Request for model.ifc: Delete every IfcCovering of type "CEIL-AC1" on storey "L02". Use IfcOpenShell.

First a look at what the model holds.

```python
import ifcopenshell
import ifcopenshell.util.element

model = ifcopenshell.open("model.ifc")
print(model.schema)
storey = next(s for s in model.by_type("IfcBuildingStorey") if s.Name == "L02")
coverings = [e for e in ifcopenshell.util.element.get_decomposition(storey) if e.is_a("IfcCovering")]
seen = {}
for e in coverings:
    element_type = ifcopenshell.util.element.get_type(e)
    name = element_type.Name if element_type not in (None, e) else None
    seen[name] = seen.get(name, 0) + 1
for name, count in sorted(seen.items(), key=str):
    print(count, "x", name)
```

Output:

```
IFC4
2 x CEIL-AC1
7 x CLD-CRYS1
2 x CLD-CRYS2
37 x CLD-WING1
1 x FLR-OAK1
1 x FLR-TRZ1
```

```python
import ifcopenshell
import ifcopenshell.api.root
import ifcopenshell.util.element

model = ifcopenshell.open("model.ifc")

storey = next(s for s in model.by_type("IfcBuildingStorey") if s.Name == "L02")
coverings = [e for e in ifcopenshell.util.element.get_decomposition(storey) if e.is_a("IfcCovering")]
targets = [e for e in coverings if (t := ifcopenshell.util.element.get_type(e)) not in (None, e) and t.Name == "CEIL-AC1"]

for e in targets:
    ifcopenshell.api.root.remove_product(model, product=e)
print(len(targets), "removed")

model.write("model-out.ifc")
```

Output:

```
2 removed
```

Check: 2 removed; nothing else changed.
